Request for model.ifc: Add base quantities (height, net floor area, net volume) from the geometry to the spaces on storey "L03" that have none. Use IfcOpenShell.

First a look at what the model holds.

```python
import ifcopenshell
import ifcopenshell.util.element
import ifcopenshell.util.unit

model = ifcopenshell.open("model.ifc")
print(model.schema)
for unit_type in ("LENGTHUNIT", "AREAUNIT", "VOLUMEUNIT"):
    print(unit_type, ifcopenshell.util.unit.calculate_unit_scale(model, unit_type))
storey = next(s for s in model.by_type("IfcBuildingStorey") if s.Name == "L03")
spaces = [e for e in ifcopenshell.util.element.get_decomposition(storey) if e.is_a("IfcSpace")]
for e in sorted(spaces, key=lambda e: e.id()):
    print(e.id(), e.is_a(), e.Name, list(ifcopenshell.util.element.get_psets(e, qtos_only=True)), sep=" | ")
```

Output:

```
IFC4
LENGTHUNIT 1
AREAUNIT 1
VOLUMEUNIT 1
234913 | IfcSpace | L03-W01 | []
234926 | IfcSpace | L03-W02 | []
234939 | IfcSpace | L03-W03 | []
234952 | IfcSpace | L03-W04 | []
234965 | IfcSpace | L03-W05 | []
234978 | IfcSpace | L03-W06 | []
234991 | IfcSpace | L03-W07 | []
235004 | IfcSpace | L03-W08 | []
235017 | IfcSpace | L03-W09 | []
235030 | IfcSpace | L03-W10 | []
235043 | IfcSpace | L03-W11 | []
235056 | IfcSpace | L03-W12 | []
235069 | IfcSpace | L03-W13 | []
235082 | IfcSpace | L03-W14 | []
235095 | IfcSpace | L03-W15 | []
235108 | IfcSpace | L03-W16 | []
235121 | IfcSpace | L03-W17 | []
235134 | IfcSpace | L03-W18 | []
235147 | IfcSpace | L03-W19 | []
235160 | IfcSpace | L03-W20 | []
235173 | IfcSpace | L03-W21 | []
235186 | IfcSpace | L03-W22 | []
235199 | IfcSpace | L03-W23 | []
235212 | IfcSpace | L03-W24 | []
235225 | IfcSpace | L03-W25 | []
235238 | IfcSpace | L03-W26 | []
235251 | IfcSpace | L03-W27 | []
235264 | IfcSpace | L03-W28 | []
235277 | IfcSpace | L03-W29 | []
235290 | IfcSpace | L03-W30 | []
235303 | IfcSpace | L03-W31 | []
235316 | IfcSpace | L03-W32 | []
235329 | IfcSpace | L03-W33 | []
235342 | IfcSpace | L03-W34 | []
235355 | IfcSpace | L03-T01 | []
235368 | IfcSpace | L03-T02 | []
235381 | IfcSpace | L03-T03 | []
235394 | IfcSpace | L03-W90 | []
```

```python
import ifcopenshell
import ifcopenshell.api.pset
import ifcopenshell.geom
import ifcopenshell.util.element
import ifcopenshell.util.shape
import ifcopenshell.util.unit

model = ifcopenshell.open("model.ifc")
unit_scale = ifcopenshell.util.unit.calculate_unit_scale(model)
area_scale = ifcopenshell.util.unit.calculate_unit_scale(model, "AREAUNIT")
volume_scale = ifcopenshell.util.unit.calculate_unit_scale(model, "VOLUMEUNIT")
settings = ifcopenshell.geom.settings()

storey = next(s for s in model.by_type("IfcBuildingStorey") if s.Name == "L03")
spaces = [e for e in ifcopenshell.util.element.get_decomposition(storey) if e.is_a("IfcSpace")]

for e in sorted(spaces, key=lambda e: e.id()):
    if ifcopenshell.util.element.get_psets(e, qtos_only=True, should_inherit=False):
        continue
    # Geometry comes back in metres, in the element's own axes.
    shape = ifcopenshell.geom.create_shape(settings, e)
    values = {
        "Height": ifcopenshell.util.shape.get_z(shape.geometry) / unit_scale,
        "NetFloorArea": ifcopenshell.util.shape.get_footprint_area(shape.geometry) / area_scale,
        "NetVolume": ifcopenshell.util.shape.get_volume(shape.geometry) / volume_scale,
    }
    qto = ifcopenshell.api.pset.add_qto(model, product=e, name="Qto_SpaceBaseQuantities")
    ifcopenshell.api.pset.edit_qto(model, qto=qto, properties=values)
    print(e.id(), {k: round(v, 3) for k, v in values.items()})

model.write("model_edited.ifc")
```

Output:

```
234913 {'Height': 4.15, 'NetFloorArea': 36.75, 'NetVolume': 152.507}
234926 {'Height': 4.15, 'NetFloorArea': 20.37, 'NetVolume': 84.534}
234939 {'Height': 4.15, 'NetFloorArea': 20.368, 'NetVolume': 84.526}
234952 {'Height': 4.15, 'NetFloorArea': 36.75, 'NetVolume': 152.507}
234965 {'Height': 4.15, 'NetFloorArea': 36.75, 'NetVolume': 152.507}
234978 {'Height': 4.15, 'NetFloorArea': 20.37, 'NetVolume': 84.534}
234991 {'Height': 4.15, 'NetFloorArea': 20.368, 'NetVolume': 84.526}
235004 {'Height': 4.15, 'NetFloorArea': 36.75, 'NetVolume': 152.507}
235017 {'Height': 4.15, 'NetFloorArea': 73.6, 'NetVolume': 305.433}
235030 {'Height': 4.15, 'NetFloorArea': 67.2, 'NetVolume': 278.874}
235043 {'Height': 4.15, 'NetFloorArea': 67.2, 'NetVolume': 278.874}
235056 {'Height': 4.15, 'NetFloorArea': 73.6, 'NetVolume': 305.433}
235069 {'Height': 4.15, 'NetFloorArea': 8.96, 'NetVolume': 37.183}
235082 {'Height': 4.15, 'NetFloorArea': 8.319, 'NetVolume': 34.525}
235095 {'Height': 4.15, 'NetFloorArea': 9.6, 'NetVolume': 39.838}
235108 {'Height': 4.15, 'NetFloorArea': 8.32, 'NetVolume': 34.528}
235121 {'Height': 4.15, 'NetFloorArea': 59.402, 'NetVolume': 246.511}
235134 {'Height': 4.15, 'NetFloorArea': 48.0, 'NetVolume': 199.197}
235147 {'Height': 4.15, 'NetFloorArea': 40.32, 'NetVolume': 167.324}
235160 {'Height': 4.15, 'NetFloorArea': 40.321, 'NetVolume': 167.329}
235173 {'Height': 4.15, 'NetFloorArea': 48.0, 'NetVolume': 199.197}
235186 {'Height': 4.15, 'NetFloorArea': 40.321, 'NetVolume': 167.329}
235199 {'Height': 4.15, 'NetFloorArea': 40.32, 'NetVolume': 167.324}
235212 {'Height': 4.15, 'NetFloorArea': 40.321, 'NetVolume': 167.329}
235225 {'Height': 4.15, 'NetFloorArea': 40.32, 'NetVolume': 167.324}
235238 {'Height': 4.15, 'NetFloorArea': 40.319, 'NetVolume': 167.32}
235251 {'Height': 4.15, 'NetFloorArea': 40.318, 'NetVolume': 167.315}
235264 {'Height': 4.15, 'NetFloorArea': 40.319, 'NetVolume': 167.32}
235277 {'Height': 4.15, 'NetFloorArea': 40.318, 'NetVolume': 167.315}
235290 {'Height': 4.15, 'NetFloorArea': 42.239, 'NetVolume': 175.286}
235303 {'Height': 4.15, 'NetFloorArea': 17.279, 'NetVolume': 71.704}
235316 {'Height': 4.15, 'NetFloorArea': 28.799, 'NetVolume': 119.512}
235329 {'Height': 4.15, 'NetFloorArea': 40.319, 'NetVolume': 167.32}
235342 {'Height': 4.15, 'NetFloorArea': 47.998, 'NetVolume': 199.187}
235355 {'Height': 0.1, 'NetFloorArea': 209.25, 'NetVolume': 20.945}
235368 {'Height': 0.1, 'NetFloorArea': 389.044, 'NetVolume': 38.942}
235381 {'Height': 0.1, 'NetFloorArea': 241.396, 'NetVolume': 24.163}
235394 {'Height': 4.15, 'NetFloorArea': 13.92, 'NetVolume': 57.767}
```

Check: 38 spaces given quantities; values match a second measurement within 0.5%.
